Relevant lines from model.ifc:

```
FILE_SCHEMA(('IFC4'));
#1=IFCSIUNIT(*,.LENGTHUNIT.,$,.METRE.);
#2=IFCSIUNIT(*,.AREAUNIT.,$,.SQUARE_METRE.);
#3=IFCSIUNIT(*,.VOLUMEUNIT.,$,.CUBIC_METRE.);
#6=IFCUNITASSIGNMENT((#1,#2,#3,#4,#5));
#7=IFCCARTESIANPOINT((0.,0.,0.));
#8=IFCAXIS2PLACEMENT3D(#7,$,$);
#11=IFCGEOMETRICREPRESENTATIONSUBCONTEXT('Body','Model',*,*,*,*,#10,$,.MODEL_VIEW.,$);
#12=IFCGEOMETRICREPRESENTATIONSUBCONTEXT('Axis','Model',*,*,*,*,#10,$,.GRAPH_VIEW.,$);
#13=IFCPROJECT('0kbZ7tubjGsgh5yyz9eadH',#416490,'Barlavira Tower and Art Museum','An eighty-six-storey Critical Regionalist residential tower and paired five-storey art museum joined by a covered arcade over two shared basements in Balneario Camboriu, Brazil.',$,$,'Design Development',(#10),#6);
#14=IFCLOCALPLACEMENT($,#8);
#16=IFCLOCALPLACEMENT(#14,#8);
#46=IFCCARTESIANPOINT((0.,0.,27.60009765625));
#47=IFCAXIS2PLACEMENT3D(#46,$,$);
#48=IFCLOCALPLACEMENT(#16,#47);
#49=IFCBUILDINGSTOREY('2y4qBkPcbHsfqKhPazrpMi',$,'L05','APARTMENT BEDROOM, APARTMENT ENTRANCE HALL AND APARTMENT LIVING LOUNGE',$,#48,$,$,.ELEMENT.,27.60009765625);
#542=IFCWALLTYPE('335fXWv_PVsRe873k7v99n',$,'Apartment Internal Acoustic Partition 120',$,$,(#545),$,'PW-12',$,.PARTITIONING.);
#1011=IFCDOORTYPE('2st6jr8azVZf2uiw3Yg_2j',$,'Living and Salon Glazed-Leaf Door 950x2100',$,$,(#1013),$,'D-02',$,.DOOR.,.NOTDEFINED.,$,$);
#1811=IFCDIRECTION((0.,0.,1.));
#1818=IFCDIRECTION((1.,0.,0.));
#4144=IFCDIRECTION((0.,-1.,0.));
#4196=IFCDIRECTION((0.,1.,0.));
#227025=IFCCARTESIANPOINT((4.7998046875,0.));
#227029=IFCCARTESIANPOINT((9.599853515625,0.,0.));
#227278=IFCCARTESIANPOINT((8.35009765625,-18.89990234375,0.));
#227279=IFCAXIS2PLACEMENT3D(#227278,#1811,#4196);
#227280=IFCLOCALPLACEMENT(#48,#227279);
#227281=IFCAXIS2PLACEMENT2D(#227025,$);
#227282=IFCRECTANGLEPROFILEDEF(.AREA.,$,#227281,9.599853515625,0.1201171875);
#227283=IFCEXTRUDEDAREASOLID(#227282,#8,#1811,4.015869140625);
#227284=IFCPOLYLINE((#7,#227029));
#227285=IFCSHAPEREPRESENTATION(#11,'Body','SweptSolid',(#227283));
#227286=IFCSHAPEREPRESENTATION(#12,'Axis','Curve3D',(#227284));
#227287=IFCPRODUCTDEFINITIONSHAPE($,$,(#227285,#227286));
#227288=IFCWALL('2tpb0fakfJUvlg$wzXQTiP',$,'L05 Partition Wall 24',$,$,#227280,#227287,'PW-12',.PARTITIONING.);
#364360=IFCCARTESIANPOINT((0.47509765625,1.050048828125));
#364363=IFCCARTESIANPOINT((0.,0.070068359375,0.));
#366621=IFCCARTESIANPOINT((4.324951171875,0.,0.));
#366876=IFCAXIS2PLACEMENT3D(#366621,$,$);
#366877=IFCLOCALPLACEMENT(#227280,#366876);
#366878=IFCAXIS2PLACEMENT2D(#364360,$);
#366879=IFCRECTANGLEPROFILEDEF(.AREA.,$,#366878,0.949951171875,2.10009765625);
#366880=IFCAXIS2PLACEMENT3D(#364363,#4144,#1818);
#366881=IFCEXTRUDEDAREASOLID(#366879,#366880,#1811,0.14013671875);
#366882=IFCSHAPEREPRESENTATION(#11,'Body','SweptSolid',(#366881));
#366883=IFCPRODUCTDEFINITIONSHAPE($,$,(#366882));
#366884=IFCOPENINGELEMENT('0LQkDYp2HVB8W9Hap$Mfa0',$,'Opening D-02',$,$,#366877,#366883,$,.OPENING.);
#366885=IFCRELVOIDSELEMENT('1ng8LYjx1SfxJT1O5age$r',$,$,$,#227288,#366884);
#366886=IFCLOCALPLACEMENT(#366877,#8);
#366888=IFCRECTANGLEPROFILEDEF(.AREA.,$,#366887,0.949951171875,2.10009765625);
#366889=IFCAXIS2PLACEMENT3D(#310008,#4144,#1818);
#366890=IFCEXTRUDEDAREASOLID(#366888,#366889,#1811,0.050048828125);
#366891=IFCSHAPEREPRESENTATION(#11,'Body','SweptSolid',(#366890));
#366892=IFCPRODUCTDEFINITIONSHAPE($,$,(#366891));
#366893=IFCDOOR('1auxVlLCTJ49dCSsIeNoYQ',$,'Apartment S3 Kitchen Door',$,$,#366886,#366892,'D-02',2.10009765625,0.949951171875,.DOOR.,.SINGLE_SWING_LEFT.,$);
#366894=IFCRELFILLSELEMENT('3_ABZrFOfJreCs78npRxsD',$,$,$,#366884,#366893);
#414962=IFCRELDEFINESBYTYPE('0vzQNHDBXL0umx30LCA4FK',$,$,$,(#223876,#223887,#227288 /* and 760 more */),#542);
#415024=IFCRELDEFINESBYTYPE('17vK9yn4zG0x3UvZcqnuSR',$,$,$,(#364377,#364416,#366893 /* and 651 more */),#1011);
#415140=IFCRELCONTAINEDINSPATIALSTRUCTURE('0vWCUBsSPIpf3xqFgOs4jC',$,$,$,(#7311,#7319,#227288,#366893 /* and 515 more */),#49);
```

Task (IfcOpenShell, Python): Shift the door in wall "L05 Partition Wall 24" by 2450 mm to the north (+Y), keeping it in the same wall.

```python
import ifcopenshell
import ifcopenshell.api.geometry
import ifcopenshell.util.placement
import ifcopenshell.util.unit

model = ifcopenshell.open("model.ifc")
unit_scale = ifcopenshell.util.unit.calculate_unit_scale(model)

door = model.by_id(366893)
opening = door.FillsVoids[0].RelatingOpeningElement
wall = opening.VoidsElements[0].RelatingBuildingElement

wall_matrix = ifcopenshell.util.placement.get_local_placement(wall.ObjectPlacement)
shift = wall_matrix[:3, 0] * 2.45 / unit_scale
before = ifcopenshell.util.placement.get_local_placement(door.ObjectPlacement)[:3, 3].copy()

# The door is placed relative to its opening, so it follows when the opening moves.
matrix = ifcopenshell.util.placement.get_local_placement(opening.ObjectPlacement)
matrix[:3, 3] += shift
ifcopenshell.api.geometry.edit_object_placement(
    model, product=opening, matrix=matrix, is_si=False, should_transform_children=True
)

after = ifcopenshell.util.placement.get_local_placement(door.ObjectPlacement)[:3, 3]
print("door moved by", (after - before).round(3) + 0.0)

model.write("model-out.ifc")
```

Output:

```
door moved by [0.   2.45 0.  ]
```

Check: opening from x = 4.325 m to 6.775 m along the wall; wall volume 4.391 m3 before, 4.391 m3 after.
